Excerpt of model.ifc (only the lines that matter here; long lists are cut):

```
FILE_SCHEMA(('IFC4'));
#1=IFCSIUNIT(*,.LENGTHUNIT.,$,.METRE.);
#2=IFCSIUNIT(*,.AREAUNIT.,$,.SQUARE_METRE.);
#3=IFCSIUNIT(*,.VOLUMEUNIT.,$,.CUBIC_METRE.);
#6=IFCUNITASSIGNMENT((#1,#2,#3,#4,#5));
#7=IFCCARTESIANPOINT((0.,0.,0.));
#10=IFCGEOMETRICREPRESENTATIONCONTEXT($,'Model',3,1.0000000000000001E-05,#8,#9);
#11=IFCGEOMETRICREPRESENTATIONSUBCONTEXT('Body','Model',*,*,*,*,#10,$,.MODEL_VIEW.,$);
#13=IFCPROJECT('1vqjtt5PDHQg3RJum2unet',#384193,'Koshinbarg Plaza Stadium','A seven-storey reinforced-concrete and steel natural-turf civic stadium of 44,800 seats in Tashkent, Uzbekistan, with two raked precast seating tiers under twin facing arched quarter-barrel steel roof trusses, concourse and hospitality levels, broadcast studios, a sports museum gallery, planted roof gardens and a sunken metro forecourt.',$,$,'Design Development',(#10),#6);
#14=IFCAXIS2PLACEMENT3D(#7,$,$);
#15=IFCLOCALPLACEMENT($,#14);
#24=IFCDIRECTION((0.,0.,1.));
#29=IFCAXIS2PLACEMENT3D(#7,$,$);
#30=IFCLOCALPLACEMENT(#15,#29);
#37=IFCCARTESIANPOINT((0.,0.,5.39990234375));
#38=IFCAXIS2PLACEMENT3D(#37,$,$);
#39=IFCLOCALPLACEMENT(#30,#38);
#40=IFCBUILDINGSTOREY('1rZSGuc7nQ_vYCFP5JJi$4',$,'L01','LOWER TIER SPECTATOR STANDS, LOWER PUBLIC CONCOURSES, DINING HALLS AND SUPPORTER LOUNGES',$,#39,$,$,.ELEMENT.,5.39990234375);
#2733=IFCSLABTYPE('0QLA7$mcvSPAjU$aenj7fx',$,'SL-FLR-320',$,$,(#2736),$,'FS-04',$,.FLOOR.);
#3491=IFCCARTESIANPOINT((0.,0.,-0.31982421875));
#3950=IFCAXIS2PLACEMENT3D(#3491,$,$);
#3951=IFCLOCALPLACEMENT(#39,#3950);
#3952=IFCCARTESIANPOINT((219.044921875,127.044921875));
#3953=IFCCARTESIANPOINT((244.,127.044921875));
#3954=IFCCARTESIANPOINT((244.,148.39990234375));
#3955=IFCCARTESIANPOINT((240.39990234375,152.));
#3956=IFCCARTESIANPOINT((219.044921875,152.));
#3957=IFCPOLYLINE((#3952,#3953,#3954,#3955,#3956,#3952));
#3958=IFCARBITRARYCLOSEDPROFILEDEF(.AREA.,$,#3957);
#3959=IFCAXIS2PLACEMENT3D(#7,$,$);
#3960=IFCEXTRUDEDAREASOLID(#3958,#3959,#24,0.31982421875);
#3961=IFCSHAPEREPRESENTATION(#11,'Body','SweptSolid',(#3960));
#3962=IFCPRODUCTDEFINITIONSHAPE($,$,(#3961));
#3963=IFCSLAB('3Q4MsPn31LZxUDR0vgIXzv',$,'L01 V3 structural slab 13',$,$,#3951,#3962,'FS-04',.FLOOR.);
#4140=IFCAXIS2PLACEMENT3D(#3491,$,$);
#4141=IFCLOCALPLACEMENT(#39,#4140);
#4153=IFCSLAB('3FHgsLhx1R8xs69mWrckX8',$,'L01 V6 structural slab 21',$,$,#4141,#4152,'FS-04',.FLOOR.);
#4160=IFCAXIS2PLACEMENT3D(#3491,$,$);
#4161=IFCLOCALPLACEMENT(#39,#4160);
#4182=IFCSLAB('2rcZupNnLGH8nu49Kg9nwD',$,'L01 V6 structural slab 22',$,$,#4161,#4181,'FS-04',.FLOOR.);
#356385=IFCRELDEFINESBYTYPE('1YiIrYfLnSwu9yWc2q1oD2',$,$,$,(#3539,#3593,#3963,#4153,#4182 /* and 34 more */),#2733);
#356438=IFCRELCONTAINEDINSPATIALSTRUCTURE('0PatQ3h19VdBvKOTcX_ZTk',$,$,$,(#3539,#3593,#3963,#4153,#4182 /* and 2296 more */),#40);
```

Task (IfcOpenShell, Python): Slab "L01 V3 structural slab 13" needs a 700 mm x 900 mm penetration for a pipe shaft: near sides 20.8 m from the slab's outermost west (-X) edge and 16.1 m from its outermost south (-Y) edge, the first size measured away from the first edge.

```python
import numpy as np
import ifcopenshell
import ifcopenshell.api.feature
import ifcopenshell.api.geometry
import ifcopenshell.api.root
import ifcopenshell.geom
import ifcopenshell.util.placement
import ifcopenshell.util.representation
import ifcopenshell.util.shape
import ifcopenshell.util.unit

model = ifcopenshell.open("model.ifc")
unit_scale = ifcopenshell.util.unit.calculate_unit_scale(model)
settings = ifcopenshell.geom.settings()


def volume(element):
    """Net volume in cubic metres, openings subtracted."""
    shape = ifcopenshell.geom.create_shape(settings, element)
    return ifcopenshell.util.shape.get_volume(shape.geometry)


slab = model.by_guid("3Q4MsPn31LZxUDR0vgIXzv")
before = volume(slab)

# Extent in the slab's own axes, in metres. The edges named are its -X and -Y sides.
slab_shape = ifcopenshell.geom.create_shape(settings, slab)
vertices = ifcopenshell.util.shape.get_vertices(slab_shape.geometry)
x_min, y_min, bottom = vertices.min(axis=0)
top = vertices[:, 2].max()

opening = ifcopenshell.api.root.create_entity(model, ifc_class="IfcOpeningElement", name="Pipe shaft opening", predefined_type="OPENING")
context = ifcopenshell.util.representation.get_context(model, "Model", "Body", "MODEL_VIEW")
width, depth = 0.7, 0.9
outline = [(0.0, 0.0), (width, 0.0), (width, depth), (0.0, depth), (0.0, 0.0)]
# Overshoot both faces by 50 mm so the cut is clean.
shape = ifcopenshell.api.geometry.add_slab_representation(
    model, context=context, depth=top - bottom + 0.1, polyline=outline
)
ifcopenshell.api.geometry.assign_representation(model, product=opening, representation=shape)

matrix = ifcopenshell.util.placement.get_local_placement(slab.ObjectPlacement)
matrix[:, 3] = matrix @ np.append(np.array([x_min + 20.8, y_min + 16.1, bottom - 0.05]) / unit_scale, 1.0)
ifcopenshell.api.geometry.edit_object_placement(model, product=opening, matrix=matrix, is_si=False)
ifcopenshell.api.feature.add_feature(model, feature=opening, element=slab)

after = volume(slab)

print(f"slab volume {before:.3f} -> {after:.3f} m3")

model.write("model_rev.ifc")
```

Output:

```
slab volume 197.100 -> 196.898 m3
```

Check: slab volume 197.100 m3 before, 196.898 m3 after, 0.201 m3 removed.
